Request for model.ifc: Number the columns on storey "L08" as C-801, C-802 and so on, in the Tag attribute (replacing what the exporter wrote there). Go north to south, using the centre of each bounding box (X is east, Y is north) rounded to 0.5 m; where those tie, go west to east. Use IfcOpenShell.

First a look at what the model holds.

```python
import ifcopenshell
import ifcopenshell.util.element
import ifcopenshell.util.placement

model = ifcopenshell.open("model.ifc")
print(model.schema)
storey = next(s for s in model.by_type("IfcBuildingStorey") if s.Name == "L08")
columns = [e for e in ifcopenshell.util.element.get_decomposition(storey) if e.is_a("IfcColumn")]
for e in sorted(columns, key=lambda e: e.id()):
    origin = ifcopenshell.util.placement.get_local_placement(e.ObjectPlacement)[:3, 3]
    print(e.id(), e.Tag, e.Name, origin.round(2) + 0.0, sep=" | ")
```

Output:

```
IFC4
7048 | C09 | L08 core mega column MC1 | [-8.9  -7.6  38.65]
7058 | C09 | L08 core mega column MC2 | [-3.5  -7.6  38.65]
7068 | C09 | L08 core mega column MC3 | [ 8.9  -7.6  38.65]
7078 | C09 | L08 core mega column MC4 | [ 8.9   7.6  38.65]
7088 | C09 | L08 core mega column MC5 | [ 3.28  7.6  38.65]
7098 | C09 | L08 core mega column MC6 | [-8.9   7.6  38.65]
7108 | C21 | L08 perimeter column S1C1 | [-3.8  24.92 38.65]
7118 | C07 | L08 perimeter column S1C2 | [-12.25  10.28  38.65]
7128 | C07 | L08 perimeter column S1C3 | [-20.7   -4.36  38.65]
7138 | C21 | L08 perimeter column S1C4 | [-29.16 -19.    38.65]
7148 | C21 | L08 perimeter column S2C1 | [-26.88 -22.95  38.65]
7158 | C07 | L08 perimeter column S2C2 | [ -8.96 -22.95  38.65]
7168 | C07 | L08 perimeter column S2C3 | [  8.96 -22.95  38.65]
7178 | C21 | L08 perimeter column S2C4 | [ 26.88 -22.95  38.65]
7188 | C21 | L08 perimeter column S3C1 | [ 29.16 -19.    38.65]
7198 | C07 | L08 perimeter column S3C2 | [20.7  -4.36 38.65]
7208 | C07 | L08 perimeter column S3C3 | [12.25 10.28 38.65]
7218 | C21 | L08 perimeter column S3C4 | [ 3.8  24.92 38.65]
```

```python
import ifcopenshell
import ifcopenshell.geom
import ifcopenshell.util.element
import ifcopenshell.util.shape

model = ifcopenshell.open("model.ifc")
settings = ifcopenshell.geom.settings()
settings.set("use-world-coords", True)


def centre(element):
    shape = ifcopenshell.geom.create_shape(settings, element)
    return ifcopenshell.util.shape.get_bbox_centroid(shape.geometry)


storey = next(s for s in model.by_type("IfcBuildingStorey") if s.Name == "L08")
columns = [e for e in ifcopenshell.util.element.get_decomposition(storey) if e.is_a("IfcColumn")]

# Insertion points can sit at a corner or the storey origin, so sort by the geometry (in metres).
centres = {e: centre(e) for e in columns}
columns.sort(key=lambda e: (-round(centres[e][1] / 0.5), centres[e][0]))

for i, e in enumerate(columns, start=1):
    number = f"C-8{i:02d}"
    e.Tag = number
    print(e.id(), number)

model.write("model_rev.ifc")
```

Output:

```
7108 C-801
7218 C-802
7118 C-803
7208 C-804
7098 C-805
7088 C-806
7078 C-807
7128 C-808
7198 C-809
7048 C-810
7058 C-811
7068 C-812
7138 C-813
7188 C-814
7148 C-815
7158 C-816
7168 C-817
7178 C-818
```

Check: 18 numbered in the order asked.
